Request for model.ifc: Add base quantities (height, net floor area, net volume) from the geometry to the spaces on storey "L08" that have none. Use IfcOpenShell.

First a look at what the model holds.

```python
import ifcopenshell
import ifcopenshell.util.element
import ifcopenshell.util.unit

model = ifcopenshell.open("model.ifc")
print(model.schema)
for unit_type in ("LENGTHUNIT", "AREAUNIT", "VOLUMEUNIT"):
    print(unit_type, ifcopenshell.util.unit.calculate_unit_scale(model, unit_type))
storey = next(s for s in model.by_type("IfcBuildingStorey") if s.Name == "L08")
spaces = [e for e in ifcopenshell.util.element.get_decomposition(storey) if e.is_a("IfcSpace")]
for e in sorted(spaces, key=lambda e: e.id()):
    print(e.id(), e.is_a(), e.Name, list(ifcopenshell.util.element.get_psets(e, qtos_only=True)), sep=" | ")
```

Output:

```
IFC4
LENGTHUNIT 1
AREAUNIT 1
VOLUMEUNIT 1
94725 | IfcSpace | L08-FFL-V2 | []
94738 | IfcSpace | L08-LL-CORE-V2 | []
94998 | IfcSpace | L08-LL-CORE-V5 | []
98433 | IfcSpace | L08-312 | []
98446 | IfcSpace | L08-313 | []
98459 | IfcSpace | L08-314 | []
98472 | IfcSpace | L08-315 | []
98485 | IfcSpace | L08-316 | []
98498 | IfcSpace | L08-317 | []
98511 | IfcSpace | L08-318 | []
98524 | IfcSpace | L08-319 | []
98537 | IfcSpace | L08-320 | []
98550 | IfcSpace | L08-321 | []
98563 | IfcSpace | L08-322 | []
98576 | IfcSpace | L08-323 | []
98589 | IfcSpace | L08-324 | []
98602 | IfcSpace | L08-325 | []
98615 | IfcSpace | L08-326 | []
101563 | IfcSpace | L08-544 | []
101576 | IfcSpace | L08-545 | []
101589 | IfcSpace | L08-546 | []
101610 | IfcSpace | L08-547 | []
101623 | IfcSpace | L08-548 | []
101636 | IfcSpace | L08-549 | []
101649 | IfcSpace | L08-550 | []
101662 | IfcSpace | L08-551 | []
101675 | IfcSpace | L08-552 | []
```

```python
import ifcopenshell
import ifcopenshell.api.pset
import ifcopenshell.geom
import ifcopenshell.util.element
import ifcopenshell.util.shape
import ifcopenshell.util.unit

model = ifcopenshell.open("model.ifc")
unit_scale = ifcopenshell.util.unit.calculate_unit_scale(model)
area_scale = ifcopenshell.util.unit.calculate_unit_scale(model, "AREAUNIT")
volume_scale = ifcopenshell.util.unit.calculate_unit_scale(model, "VOLUMEUNIT")
settings = ifcopenshell.geom.settings()

storey = next(s for s in model.by_type("IfcBuildingStorey") if s.Name == "L08")
spaces = [e for e in ifcopenshell.util.element.get_decomposition(storey) if e.is_a("IfcSpace")]

for e in sorted(spaces, key=lambda e: e.id()):
    if ifcopenshell.util.element.get_psets(e, qtos_only=True, should_inherit=False):
        continue
    # Geometry comes back in metres, in the element's own axes.
    shape = ifcopenshell.geom.create_shape(settings, e)
    values = {
        "Height": ifcopenshell.util.shape.get_z(shape.geometry) / unit_scale,
        "NetFloorArea": ifcopenshell.util.shape.get_footprint_area(shape.geometry) / area_scale,
        "NetVolume": ifcopenshell.util.shape.get_volume(shape.geometry) / volume_scale,
    }
    qto = ifcopenshell.api.pset.add_qto(model, product=e, name="Qto_SpaceBaseQuantities")
    ifcopenshell.api.pset.edit_qto(model, qto=qto, properties=values)
    print(e.id(), {k: round(v, 3) for k, v in values.items()})

model.write("model-out.ifc")
```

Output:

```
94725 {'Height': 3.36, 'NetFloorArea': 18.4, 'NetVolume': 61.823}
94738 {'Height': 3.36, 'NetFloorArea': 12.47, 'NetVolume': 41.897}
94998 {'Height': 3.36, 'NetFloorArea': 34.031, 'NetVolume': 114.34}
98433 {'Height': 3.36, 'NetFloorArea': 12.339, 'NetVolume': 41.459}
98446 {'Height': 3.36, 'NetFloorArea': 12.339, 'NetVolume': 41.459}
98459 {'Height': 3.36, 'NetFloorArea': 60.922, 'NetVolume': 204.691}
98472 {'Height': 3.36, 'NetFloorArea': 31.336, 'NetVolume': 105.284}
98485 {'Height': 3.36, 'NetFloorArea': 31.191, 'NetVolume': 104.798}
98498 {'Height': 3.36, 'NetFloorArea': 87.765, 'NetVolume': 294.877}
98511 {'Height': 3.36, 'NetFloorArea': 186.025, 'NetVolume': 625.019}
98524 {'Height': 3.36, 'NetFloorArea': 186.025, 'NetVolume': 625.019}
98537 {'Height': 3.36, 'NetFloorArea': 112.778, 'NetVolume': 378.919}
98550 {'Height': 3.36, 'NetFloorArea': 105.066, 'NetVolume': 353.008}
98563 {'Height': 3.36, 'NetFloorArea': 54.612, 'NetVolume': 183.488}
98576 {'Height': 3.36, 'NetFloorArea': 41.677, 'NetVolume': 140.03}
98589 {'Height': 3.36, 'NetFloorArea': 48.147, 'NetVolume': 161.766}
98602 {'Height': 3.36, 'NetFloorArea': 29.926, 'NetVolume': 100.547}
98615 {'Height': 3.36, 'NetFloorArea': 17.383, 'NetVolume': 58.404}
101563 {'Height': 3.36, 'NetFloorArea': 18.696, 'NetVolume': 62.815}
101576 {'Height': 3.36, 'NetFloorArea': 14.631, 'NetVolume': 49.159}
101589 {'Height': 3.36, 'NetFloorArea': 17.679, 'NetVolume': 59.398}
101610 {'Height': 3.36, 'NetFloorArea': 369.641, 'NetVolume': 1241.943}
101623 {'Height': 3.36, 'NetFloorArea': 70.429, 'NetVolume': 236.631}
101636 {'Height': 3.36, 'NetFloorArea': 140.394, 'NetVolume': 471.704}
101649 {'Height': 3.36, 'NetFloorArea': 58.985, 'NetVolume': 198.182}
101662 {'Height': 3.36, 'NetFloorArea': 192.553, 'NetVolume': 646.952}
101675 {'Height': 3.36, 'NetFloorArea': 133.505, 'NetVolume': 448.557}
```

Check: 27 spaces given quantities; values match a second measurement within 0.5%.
